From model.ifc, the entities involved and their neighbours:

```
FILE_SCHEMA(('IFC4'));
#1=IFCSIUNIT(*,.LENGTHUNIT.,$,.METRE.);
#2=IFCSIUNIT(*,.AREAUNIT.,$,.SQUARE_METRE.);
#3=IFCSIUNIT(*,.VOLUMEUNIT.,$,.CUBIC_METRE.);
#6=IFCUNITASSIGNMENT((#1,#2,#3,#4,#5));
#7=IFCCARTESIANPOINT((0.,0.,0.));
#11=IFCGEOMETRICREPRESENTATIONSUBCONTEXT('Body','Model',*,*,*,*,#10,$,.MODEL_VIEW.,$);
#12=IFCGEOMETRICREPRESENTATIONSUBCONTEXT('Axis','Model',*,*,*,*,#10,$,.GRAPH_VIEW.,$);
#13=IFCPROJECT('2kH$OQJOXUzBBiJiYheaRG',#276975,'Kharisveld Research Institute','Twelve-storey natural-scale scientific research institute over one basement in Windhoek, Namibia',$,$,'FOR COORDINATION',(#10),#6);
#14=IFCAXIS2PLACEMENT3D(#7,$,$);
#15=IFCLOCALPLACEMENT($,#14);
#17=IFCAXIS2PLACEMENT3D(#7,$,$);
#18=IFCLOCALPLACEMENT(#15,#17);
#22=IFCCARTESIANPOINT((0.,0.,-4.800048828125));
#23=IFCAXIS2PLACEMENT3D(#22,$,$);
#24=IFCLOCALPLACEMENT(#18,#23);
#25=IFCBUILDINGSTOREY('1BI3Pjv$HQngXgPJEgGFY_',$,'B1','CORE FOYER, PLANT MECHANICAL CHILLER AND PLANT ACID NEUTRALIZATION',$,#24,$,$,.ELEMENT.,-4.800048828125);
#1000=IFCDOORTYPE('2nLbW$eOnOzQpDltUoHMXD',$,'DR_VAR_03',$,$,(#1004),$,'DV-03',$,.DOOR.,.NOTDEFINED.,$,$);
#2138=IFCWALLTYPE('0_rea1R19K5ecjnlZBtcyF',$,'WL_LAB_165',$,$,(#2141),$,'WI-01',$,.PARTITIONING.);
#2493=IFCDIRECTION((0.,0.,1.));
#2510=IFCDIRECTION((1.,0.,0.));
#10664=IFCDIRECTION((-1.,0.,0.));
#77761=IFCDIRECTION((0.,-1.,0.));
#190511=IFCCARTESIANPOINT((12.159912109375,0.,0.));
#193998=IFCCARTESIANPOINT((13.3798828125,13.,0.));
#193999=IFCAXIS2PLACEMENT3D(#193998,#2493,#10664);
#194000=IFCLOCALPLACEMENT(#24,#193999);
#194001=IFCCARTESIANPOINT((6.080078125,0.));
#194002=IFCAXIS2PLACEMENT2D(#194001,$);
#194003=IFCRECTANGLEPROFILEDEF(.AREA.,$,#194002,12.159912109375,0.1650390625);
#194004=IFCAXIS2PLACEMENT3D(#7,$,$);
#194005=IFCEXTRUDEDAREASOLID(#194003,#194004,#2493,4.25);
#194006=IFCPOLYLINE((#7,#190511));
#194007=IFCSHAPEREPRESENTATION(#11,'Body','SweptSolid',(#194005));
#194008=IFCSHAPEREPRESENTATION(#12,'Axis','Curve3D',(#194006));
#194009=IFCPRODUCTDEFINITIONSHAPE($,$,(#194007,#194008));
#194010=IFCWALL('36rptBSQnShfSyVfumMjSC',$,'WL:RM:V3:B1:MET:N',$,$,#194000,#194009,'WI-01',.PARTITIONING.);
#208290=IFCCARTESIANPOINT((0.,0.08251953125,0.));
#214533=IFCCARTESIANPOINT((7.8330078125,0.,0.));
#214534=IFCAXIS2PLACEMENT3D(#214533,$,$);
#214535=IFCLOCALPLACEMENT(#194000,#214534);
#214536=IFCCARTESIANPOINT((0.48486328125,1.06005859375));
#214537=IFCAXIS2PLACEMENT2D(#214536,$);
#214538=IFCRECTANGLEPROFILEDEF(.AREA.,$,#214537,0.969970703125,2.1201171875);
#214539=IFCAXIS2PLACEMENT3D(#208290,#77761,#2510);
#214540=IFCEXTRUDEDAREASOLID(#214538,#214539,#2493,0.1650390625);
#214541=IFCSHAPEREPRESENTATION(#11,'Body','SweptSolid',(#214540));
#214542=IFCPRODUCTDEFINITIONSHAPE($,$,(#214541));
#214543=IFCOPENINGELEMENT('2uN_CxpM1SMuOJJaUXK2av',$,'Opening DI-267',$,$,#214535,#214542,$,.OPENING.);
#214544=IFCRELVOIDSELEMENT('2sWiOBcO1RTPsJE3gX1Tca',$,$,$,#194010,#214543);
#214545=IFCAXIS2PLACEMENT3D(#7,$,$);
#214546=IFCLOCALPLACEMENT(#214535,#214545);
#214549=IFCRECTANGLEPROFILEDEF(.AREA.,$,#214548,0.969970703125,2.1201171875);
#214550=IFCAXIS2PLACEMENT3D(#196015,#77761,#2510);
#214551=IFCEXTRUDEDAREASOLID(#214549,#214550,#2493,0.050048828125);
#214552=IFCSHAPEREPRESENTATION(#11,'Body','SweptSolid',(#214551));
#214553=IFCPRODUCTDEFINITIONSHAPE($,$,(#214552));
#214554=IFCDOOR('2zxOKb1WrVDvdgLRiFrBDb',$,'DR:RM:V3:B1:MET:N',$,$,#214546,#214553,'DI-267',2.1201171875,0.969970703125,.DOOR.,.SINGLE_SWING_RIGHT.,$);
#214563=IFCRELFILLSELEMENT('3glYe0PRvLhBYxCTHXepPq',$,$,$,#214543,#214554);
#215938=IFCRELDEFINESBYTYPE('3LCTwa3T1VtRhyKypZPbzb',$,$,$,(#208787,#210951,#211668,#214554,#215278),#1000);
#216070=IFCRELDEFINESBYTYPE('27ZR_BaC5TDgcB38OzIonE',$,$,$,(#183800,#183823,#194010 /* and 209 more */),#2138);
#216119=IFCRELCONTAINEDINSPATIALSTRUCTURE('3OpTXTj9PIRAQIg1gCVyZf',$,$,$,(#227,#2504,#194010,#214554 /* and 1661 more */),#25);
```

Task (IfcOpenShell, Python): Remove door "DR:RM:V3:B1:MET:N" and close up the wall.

```python
import ifcopenshell
import ifcopenshell.api.feature
import ifcopenshell.api.root
import ifcopenshell.geom
import ifcopenshell.util.shape

model = ifcopenshell.open("model.ifc")
settings = ifcopenshell.geom.settings()


def volume(element):
    """Net volume in cubic metres, openings subtracted."""
    shape = ifcopenshell.geom.create_shape(settings, element)
    return ifcopenshell.util.shape.get_volume(shape.geometry)


door = model.by_guid("2zxOKb1WrVDvdgLRiFrBDb")
opening = door.FillsVoids[0].RelatingOpeningElement
wall = opening.VoidsElements[0].RelatingBuildingElement
before = volume(wall)

ifcopenshell.api.root.remove_product(model, product=door)
ifcopenshell.api.feature.remove_feature(model, feature=opening)

after = volume(wall)

print(f"wall volume {before:.3f} -> {after:.3f} m3")

model.write("model_updated.ifc")
```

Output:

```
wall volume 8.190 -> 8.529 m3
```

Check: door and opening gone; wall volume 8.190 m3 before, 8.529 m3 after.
